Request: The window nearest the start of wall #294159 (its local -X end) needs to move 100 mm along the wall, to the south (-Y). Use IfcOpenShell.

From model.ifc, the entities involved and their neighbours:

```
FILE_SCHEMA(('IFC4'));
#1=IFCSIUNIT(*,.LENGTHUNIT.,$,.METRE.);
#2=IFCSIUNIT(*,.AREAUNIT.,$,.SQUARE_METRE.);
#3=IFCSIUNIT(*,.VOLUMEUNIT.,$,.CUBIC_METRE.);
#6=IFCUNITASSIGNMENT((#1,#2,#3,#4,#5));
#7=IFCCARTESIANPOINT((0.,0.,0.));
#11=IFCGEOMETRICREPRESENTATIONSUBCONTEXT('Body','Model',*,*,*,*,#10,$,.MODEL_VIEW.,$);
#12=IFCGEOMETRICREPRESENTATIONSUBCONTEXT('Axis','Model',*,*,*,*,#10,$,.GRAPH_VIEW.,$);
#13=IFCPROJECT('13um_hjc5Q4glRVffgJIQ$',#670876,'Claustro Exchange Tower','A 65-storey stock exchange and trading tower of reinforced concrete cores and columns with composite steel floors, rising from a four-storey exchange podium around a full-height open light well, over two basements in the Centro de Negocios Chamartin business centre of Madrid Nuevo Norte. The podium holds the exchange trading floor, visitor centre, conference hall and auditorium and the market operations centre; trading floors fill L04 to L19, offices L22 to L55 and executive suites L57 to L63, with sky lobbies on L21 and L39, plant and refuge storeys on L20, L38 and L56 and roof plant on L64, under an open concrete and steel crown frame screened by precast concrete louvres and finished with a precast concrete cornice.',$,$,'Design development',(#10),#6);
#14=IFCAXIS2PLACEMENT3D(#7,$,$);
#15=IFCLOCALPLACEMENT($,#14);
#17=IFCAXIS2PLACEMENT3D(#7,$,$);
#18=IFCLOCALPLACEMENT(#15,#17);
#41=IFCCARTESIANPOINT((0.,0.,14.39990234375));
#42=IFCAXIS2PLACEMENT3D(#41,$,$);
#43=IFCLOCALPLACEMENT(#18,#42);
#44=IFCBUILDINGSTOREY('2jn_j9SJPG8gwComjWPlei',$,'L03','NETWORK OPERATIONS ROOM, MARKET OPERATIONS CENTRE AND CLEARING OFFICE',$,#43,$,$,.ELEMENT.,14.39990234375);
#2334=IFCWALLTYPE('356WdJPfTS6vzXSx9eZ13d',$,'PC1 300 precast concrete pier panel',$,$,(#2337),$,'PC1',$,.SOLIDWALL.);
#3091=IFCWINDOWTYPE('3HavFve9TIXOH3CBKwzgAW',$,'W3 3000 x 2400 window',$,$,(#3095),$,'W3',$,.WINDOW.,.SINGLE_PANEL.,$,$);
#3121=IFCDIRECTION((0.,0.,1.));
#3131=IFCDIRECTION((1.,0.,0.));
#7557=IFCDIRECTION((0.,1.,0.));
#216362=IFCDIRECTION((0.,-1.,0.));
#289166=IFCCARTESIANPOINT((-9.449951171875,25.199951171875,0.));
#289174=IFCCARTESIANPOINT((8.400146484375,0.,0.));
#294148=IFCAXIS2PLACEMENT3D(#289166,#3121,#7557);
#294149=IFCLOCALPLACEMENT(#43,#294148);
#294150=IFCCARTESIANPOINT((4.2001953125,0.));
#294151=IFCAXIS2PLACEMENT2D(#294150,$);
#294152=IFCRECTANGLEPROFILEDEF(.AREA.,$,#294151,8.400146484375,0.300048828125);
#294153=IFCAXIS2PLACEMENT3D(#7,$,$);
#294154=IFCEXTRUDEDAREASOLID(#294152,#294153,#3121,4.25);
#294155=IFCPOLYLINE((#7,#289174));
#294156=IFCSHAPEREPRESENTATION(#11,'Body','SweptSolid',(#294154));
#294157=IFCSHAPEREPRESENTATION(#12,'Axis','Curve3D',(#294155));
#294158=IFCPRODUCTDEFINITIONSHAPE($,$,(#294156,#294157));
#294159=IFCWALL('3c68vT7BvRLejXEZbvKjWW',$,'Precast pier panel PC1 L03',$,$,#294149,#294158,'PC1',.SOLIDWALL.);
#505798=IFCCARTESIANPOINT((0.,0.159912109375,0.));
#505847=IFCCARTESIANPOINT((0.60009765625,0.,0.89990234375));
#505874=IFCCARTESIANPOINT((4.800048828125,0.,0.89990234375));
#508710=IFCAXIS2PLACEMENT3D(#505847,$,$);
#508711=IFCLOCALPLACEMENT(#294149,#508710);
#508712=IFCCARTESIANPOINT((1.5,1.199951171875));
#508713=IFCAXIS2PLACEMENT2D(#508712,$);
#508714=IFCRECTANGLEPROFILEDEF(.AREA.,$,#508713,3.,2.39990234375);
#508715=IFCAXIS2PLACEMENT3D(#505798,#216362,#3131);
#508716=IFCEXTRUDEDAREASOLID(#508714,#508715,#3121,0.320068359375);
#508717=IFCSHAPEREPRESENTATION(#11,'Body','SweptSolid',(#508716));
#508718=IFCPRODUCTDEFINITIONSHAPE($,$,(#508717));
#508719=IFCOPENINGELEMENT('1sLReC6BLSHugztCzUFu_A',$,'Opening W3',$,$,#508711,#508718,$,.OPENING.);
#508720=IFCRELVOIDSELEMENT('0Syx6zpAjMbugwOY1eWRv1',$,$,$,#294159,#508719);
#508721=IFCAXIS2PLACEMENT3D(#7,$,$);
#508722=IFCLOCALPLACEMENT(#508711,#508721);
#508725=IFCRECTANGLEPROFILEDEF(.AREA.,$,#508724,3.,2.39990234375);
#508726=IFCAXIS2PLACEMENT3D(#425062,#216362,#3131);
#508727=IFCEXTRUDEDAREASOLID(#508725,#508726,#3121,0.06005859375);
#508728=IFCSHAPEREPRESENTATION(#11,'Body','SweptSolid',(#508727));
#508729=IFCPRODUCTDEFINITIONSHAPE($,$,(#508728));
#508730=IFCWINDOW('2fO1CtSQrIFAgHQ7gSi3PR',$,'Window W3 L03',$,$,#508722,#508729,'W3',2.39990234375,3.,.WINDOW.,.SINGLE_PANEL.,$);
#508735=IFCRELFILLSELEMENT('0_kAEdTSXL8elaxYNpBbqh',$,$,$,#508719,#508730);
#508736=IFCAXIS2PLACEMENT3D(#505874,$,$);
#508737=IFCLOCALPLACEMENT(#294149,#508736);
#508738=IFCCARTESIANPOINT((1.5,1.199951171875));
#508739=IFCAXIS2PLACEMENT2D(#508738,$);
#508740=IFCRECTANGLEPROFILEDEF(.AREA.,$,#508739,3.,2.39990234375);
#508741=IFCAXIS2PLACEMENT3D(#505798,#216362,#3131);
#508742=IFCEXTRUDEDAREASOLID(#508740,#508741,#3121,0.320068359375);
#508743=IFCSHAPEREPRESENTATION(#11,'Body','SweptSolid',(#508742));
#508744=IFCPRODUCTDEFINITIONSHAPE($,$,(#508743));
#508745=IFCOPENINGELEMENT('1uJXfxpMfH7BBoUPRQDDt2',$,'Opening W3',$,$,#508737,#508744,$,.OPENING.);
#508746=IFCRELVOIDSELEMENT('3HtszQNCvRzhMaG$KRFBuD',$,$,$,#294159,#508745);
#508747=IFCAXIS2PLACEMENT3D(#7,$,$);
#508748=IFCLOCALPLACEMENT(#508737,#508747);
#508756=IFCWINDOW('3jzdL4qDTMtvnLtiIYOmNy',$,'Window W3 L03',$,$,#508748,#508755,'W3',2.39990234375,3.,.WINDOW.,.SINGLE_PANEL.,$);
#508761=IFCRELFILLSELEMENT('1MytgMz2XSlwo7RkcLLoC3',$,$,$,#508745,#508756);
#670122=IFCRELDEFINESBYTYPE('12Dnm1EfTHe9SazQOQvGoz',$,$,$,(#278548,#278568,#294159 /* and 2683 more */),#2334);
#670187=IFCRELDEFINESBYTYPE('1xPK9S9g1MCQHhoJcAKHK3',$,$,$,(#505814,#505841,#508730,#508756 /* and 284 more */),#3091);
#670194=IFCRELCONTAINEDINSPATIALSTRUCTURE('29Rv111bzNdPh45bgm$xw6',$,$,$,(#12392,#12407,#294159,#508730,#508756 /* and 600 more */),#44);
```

```python
import ifcopenshell
import ifcopenshell.api.geometry
import ifcopenshell.util.placement

model = ifcopenshell.open("model.ifc")

window = model.by_guid("2fO1CtSQrIFAgHQ7gSi3PR")
opening = window.FillsVoids[0].RelatingOpeningElement
wall = opening.VoidsElements[0].RelatingBuildingElement

wall_matrix = ifcopenshell.util.placement.get_local_placement(wall.ObjectPlacement)
shift = wall_matrix[:3, 0] * -0.1
before = ifcopenshell.util.placement.get_local_placement(window.ObjectPlacement)[:3, 3].copy()

# The window is placed relative to its opening, so it follows when the opening moves.
matrix = ifcopenshell.util.placement.get_local_placement(opening.ObjectPlacement)
matrix[:3, 3] += shift
ifcopenshell.api.geometry.edit_object_placement(
    model, product=opening, matrix=matrix, is_si=False, should_transform_children=True
)

after = ifcopenshell.util.placement.get_local_placement(window.ObjectPlacement)[:3, 3]
print("window moved by", (after - before).round(3) + 0.0)

model.write("model_edited.ifc")
```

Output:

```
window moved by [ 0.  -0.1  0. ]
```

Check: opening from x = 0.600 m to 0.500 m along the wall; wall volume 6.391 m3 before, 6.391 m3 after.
